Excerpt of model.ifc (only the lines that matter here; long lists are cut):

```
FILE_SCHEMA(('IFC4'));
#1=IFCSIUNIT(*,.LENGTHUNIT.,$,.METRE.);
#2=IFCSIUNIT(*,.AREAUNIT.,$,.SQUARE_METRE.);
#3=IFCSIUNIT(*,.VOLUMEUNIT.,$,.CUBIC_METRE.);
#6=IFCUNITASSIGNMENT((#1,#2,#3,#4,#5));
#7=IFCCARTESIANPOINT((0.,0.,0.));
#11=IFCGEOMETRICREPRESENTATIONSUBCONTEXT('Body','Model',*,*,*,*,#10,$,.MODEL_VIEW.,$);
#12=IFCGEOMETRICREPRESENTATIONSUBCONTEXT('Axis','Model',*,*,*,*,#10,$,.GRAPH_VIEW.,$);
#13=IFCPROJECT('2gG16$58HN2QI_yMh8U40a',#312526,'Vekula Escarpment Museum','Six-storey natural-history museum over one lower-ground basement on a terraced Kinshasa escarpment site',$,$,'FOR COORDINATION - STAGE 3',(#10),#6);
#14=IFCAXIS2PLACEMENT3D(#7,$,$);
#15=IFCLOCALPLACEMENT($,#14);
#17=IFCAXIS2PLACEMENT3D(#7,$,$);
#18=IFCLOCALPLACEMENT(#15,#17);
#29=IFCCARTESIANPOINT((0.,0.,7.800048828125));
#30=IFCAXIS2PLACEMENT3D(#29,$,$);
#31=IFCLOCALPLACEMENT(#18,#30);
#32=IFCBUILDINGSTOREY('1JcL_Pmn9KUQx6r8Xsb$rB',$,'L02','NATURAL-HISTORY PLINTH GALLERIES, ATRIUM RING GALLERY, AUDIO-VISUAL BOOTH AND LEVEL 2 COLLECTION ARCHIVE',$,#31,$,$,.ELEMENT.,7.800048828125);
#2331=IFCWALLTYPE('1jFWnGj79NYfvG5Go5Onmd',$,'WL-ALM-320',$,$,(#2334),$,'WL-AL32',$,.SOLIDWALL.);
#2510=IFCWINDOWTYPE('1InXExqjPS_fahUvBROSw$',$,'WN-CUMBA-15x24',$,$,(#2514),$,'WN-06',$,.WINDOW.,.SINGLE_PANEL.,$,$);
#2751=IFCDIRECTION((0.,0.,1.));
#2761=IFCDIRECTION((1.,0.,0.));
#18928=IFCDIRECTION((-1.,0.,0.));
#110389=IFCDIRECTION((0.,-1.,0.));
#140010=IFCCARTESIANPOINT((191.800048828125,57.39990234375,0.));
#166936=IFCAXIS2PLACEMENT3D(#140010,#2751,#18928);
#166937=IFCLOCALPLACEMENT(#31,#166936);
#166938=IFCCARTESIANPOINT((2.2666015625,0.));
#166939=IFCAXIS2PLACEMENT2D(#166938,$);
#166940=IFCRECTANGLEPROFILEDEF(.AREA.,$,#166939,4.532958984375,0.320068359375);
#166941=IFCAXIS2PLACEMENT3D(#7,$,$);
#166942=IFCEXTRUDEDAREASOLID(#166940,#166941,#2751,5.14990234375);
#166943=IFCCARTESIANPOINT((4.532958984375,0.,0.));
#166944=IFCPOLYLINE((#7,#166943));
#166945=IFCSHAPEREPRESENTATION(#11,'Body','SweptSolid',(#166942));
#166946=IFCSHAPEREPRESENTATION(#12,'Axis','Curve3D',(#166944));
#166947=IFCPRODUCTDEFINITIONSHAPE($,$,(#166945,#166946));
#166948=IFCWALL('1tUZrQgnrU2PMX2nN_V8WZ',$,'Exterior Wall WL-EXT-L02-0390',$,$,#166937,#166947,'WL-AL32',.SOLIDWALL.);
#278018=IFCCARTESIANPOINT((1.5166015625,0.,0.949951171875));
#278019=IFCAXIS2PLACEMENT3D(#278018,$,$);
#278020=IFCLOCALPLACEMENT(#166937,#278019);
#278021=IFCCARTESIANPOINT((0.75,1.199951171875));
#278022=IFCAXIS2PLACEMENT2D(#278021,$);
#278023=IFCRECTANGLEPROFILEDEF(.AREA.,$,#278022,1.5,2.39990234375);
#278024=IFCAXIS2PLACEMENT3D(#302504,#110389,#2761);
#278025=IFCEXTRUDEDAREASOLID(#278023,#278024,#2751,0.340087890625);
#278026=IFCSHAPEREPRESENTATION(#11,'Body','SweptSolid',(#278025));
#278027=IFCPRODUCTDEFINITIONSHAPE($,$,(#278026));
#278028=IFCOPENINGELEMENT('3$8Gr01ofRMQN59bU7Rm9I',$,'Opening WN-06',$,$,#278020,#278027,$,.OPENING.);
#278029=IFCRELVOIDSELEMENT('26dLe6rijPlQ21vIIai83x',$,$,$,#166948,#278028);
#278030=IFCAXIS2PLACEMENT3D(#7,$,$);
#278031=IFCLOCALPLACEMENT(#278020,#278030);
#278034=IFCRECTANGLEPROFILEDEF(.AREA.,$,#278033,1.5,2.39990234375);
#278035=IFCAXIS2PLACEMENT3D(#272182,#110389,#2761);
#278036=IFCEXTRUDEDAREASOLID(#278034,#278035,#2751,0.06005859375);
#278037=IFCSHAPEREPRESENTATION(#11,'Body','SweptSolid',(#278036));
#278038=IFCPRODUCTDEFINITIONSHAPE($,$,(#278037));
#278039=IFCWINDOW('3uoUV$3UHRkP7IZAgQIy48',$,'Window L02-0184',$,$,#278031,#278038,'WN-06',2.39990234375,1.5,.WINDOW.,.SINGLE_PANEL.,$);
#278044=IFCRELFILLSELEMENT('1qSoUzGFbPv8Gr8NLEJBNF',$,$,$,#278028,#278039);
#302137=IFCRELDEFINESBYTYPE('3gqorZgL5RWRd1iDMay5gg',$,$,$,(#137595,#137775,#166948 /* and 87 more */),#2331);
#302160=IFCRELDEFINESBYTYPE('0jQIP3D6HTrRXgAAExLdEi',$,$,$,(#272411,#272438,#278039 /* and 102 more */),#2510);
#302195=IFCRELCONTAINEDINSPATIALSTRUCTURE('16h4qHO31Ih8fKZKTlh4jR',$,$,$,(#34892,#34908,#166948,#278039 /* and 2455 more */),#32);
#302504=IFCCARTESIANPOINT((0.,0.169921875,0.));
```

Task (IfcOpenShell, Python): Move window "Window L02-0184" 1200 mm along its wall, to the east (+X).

```python
import ifcopenshell
import ifcopenshell.api.geometry
import ifcopenshell.util.placement
import ifcopenshell.util.unit

model = ifcopenshell.open("model.ifc")
unit_scale = ifcopenshell.util.unit.calculate_unit_scale(model)

window = model.by_id(278039)
opening = window.FillsVoids[0].RelatingOpeningElement
wall = opening.VoidsElements[0].RelatingBuildingElement

wall_matrix = ifcopenshell.util.placement.get_local_placement(wall.ObjectPlacement)
shift = wall_matrix[:3, 0] * -1.2 / unit_scale
before = ifcopenshell.util.placement.get_local_placement(window.ObjectPlacement)[:3, 3].copy()

# The window is placed relative to its opening, so it follows when the opening moves.
matrix = ifcopenshell.util.placement.get_local_placement(opening.ObjectPlacement)
matrix[:3, 3] += shift
ifcopenshell.api.geometry.edit_object_placement(
    model, product=opening, matrix=matrix, is_si=False, should_transform_children=True
)

after = ifcopenshell.util.placement.get_local_placement(window.ObjectPlacement)[:3, 3]
print("window moved by", (after - before).round(3) + 0.0)

model.write("model_v2.ifc")
```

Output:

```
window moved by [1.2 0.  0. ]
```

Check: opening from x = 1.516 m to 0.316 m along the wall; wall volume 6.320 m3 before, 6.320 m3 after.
